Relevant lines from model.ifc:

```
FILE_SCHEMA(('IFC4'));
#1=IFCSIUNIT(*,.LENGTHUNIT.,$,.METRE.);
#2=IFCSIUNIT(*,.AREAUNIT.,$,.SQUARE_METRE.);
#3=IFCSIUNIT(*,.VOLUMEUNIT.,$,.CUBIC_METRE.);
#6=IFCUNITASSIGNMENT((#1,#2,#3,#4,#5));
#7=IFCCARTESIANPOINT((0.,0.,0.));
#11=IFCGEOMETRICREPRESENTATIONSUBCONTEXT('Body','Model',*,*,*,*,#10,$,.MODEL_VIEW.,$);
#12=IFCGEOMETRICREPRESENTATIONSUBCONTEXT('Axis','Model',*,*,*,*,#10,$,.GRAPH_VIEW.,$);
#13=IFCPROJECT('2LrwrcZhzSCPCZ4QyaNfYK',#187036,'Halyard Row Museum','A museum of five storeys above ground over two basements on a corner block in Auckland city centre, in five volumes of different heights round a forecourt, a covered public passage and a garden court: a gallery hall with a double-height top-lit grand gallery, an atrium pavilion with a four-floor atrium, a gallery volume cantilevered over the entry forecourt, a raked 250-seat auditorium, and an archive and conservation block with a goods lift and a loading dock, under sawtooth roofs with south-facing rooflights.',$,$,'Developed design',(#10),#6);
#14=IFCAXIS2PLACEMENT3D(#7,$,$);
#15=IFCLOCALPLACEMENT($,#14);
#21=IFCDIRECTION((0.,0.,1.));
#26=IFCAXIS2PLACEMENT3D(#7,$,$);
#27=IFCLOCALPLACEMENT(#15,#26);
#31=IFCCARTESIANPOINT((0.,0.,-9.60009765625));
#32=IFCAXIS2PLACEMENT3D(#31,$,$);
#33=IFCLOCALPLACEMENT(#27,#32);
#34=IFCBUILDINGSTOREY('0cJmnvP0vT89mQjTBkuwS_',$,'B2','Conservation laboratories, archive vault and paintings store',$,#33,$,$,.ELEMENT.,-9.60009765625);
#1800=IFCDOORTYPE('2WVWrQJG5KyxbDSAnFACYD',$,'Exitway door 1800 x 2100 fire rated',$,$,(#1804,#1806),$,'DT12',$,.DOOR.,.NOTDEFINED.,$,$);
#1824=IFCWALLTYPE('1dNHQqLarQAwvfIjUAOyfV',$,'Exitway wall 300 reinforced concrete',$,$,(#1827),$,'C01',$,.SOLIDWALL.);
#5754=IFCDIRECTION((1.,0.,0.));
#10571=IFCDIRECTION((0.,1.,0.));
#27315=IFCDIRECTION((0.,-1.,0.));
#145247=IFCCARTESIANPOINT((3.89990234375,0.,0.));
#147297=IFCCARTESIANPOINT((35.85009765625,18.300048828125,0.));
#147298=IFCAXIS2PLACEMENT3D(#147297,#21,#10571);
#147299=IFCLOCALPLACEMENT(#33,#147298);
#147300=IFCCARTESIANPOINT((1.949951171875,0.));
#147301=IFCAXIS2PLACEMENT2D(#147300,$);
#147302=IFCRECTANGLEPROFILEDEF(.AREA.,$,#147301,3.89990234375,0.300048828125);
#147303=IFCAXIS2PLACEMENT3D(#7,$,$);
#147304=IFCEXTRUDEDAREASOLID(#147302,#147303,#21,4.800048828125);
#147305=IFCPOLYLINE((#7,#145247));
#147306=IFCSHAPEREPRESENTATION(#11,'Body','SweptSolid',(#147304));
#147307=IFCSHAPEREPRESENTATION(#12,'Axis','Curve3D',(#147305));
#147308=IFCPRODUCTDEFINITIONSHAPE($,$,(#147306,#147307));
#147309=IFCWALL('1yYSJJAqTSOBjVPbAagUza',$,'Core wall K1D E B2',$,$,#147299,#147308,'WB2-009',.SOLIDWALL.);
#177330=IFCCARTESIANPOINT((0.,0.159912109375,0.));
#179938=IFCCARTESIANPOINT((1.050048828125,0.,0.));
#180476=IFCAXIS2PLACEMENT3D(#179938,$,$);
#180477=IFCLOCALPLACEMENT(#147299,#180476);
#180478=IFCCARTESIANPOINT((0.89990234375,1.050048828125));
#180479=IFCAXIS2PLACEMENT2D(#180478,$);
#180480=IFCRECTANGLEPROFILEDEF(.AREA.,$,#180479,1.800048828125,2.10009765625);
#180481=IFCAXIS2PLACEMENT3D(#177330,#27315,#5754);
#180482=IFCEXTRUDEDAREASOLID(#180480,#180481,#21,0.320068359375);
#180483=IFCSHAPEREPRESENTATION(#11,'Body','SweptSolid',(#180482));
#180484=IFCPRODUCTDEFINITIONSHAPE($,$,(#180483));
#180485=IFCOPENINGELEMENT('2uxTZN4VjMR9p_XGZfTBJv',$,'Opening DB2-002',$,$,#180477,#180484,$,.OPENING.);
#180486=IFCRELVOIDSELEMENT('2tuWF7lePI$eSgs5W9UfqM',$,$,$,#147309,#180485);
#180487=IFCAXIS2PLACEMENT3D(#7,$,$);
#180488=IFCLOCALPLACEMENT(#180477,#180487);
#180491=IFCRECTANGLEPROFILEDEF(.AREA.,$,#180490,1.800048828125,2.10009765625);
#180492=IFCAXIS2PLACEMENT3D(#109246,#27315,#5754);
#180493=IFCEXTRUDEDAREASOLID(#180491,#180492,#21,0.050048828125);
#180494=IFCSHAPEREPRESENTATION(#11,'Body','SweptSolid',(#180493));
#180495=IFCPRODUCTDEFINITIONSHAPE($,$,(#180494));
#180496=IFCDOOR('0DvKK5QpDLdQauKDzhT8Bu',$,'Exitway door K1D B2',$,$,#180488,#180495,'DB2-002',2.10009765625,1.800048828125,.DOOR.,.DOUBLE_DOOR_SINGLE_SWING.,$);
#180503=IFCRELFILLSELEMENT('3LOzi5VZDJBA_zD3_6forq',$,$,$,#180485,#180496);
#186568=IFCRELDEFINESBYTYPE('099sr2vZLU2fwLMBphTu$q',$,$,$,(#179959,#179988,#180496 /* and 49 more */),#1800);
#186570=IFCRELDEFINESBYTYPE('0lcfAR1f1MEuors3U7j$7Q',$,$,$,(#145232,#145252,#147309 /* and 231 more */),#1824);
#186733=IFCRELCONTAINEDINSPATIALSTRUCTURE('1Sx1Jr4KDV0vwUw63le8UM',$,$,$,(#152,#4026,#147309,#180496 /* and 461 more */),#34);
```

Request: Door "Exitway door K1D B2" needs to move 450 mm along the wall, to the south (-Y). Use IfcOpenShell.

```python
import ifcopenshell
import ifcopenshell.api.geometry
import ifcopenshell.util.placement

model = ifcopenshell.open("model.ifc")

door = model.by_guid("0DvKK5QpDLdQauKDzhT8Bu")
opening = door.FillsVoids[0].RelatingOpeningElement
wall = opening.VoidsElements[0].RelatingBuildingElement

wall_matrix = ifcopenshell.util.placement.get_local_placement(wall.ObjectPlacement)
shift = wall_matrix[:3, 0] * -0.45
before = ifcopenshell.util.placement.get_local_placement(door.ObjectPlacement)[:3, 3].copy()

# The door is placed relative to its opening, so it follows when the opening moves.
matrix = ifcopenshell.util.placement.get_local_placement(opening.ObjectPlacement)
matrix[:3, 3] += shift
ifcopenshell.api.geometry.edit_object_placement(
    model, product=opening, matrix=matrix, is_si=False, should_transform_children=True
)

after = ifcopenshell.util.placement.get_local_placement(door.ObjectPlacement)[:3, 3]
print("door moved by", (after - before).round(3) + 0.0)

model.write("model_edited.ifc")
```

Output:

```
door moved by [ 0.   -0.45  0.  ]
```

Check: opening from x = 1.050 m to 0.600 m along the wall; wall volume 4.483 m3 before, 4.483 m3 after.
